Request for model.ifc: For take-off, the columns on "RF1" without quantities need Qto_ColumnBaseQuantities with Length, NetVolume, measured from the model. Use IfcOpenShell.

First a look at what the model holds.

```python
import ifcopenshell
import ifcopenshell.util.element
import ifcopenshell.util.unit

model = ifcopenshell.open("model.ifc")
print(model.schema)
for unit_type in ("LENGTHUNIT", "AREAUNIT", "VOLUMEUNIT"):
    print(unit_type, ifcopenshell.util.unit.calculate_unit_scale(model, unit_type))
storey = next(s for s in model.by_type("IfcBuildingStorey") if s.Name == "RF1")
columns = [e for e in ifcopenshell.util.element.get_decomposition(storey) if e.is_a("IfcColumn")]
for e in sorted(columns, key=lambda e: e.id()):
    print(e.id(), e.is_a(), e.Name, list(ifcopenshell.util.element.get_psets(e, qtos_only=True)), sep=" | ")
```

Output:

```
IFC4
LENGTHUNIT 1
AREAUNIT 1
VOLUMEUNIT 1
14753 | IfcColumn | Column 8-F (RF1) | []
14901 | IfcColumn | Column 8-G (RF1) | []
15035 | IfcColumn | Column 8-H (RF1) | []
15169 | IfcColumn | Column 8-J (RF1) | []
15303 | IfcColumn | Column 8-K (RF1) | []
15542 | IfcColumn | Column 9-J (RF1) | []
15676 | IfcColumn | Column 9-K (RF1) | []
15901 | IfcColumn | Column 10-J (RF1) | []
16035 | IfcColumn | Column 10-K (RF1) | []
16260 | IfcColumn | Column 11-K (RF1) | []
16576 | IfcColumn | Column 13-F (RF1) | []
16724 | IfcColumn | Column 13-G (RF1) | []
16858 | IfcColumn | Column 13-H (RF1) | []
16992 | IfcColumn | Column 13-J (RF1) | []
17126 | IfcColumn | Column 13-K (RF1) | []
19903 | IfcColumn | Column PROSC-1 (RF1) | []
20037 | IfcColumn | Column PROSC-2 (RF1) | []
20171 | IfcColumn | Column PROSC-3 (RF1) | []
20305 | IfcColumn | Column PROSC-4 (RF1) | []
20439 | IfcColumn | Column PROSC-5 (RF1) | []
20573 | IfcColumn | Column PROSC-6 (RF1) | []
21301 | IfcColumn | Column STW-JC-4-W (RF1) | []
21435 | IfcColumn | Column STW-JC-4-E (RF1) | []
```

```python
import ifcopenshell
import ifcopenshell.api.pset
import ifcopenshell.geom
import ifcopenshell.util.element
import ifcopenshell.util.shape
import ifcopenshell.util.unit

model = ifcopenshell.open("model.ifc")
unit_scale = ifcopenshell.util.unit.calculate_unit_scale(model)
volume_scale = ifcopenshell.util.unit.calculate_unit_scale(model, "VOLUMEUNIT")
settings = ifcopenshell.geom.settings()

storey = next(s for s in model.by_type("IfcBuildingStorey") if s.Name == "RF1")
columns = [e for e in ifcopenshell.util.element.get_decomposition(storey) if e.is_a("IfcColumn")]

for e in sorted(columns, key=lambda e: e.id()):
    if ifcopenshell.util.element.get_psets(e, qtos_only=True, should_inherit=False):
        continue
    # Geometry comes back in metres, in the element's own axes.
    shape = ifcopenshell.geom.create_shape(settings, e)
    values = {
        "Length": ifcopenshell.util.shape.get_z(shape.geometry) / unit_scale,
        "NetVolume": ifcopenshell.util.shape.get_volume(shape.geometry) / volume_scale,
    }
    qto = ifcopenshell.api.pset.add_qto(model, product=e, name="Qto_ColumnBaseQuantities")
    ifcopenshell.api.pset.edit_qto(model, qto=qto, properties=values)
    print(e.id(), {k: round(v, 3) for k, v in values.items()})

model.write("model_updated.ifc")
```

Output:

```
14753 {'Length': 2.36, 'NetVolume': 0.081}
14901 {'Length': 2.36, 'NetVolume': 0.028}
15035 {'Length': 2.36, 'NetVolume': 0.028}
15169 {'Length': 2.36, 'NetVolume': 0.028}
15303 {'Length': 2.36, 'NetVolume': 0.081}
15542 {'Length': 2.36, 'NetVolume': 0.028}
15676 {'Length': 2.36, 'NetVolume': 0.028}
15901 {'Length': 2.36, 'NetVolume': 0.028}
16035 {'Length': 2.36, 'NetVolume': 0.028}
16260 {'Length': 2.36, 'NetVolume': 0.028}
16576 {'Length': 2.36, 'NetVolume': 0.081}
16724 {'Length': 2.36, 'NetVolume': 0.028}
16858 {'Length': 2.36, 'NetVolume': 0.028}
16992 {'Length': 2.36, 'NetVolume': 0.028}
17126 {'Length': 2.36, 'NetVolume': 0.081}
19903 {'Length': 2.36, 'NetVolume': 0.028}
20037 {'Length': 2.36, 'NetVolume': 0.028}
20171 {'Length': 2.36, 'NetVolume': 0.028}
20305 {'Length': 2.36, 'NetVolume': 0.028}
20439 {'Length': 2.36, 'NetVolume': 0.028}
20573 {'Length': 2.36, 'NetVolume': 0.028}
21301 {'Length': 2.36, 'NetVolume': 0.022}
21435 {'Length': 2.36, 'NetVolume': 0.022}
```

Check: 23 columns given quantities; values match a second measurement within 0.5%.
